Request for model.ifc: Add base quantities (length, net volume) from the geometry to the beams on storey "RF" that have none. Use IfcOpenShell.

First a look at what the model holds.

```python
import ifcopenshell
import ifcopenshell.util.element
import ifcopenshell.util.unit

model = ifcopenshell.open("model.ifc")
print(model.schema)
for unit_type in ("LENGTHUNIT", "AREAUNIT", "VOLUMEUNIT"):
    print(unit_type, ifcopenshell.util.unit.calculate_unit_scale(model, unit_type))
storey = next(s for s in model.by_type("IfcBuildingStorey") if s.Name == "RF")
beams = [e for e in ifcopenshell.util.element.get_decomposition(storey) if e.is_a("IfcBeam")]
for e in sorted(beams, key=lambda e: e.id()):
    print(e.id(), e.is_a(), e.Name, list(ifcopenshell.util.element.get_psets(e, qtos_only=True)), sep=" | ")
```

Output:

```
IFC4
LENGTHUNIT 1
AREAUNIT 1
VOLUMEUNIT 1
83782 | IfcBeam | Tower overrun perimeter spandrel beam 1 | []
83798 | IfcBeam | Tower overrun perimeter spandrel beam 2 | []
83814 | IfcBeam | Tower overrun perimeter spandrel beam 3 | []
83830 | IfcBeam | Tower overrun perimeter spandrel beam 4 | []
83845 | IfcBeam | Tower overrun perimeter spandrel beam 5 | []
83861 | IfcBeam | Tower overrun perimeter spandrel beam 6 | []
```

```python
import ifcopenshell
import ifcopenshell.api.pset
import ifcopenshell.geom
import ifcopenshell.util.element
import ifcopenshell.util.shape
import ifcopenshell.util.unit

model = ifcopenshell.open("model.ifc")
unit_scale = ifcopenshell.util.unit.calculate_unit_scale(model)
volume_scale = ifcopenshell.util.unit.calculate_unit_scale(model, "VOLUMEUNIT")
settings = ifcopenshell.geom.settings()

storey = next(s for s in model.by_type("IfcBuildingStorey") if s.Name == "RF")
beams = [e for e in ifcopenshell.util.element.get_decomposition(storey) if e.is_a("IfcBeam")]

for e in sorted(beams, key=lambda e: e.id()):
    if ifcopenshell.util.element.get_psets(e, qtos_only=True, should_inherit=False):
        continue
    # Geometry comes back in metres, in the element's own axes.
    shape = ifcopenshell.geom.create_shape(settings, e)
    values = {
        "Length": ifcopenshell.util.shape.get_max_xyz(shape.geometry) / unit_scale,
        "NetVolume": ifcopenshell.util.shape.get_volume(shape.geometry) / volume_scale,
    }
    qto = ifcopenshell.api.pset.add_qto(model, product=e, name="Qto_BeamBaseQuantities")
    ifcopenshell.api.pset.edit_qto(model, qto=qto, properties=values)
    print(e.id(), {k: round(v, 3) for k, v in values.items()})

model.write("model_rev.ifc")
```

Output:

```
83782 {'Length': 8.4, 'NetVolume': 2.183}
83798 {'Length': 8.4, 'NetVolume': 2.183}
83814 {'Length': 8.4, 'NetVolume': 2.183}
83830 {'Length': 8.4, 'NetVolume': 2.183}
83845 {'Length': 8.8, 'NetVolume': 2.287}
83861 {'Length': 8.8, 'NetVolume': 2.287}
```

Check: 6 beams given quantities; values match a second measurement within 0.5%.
